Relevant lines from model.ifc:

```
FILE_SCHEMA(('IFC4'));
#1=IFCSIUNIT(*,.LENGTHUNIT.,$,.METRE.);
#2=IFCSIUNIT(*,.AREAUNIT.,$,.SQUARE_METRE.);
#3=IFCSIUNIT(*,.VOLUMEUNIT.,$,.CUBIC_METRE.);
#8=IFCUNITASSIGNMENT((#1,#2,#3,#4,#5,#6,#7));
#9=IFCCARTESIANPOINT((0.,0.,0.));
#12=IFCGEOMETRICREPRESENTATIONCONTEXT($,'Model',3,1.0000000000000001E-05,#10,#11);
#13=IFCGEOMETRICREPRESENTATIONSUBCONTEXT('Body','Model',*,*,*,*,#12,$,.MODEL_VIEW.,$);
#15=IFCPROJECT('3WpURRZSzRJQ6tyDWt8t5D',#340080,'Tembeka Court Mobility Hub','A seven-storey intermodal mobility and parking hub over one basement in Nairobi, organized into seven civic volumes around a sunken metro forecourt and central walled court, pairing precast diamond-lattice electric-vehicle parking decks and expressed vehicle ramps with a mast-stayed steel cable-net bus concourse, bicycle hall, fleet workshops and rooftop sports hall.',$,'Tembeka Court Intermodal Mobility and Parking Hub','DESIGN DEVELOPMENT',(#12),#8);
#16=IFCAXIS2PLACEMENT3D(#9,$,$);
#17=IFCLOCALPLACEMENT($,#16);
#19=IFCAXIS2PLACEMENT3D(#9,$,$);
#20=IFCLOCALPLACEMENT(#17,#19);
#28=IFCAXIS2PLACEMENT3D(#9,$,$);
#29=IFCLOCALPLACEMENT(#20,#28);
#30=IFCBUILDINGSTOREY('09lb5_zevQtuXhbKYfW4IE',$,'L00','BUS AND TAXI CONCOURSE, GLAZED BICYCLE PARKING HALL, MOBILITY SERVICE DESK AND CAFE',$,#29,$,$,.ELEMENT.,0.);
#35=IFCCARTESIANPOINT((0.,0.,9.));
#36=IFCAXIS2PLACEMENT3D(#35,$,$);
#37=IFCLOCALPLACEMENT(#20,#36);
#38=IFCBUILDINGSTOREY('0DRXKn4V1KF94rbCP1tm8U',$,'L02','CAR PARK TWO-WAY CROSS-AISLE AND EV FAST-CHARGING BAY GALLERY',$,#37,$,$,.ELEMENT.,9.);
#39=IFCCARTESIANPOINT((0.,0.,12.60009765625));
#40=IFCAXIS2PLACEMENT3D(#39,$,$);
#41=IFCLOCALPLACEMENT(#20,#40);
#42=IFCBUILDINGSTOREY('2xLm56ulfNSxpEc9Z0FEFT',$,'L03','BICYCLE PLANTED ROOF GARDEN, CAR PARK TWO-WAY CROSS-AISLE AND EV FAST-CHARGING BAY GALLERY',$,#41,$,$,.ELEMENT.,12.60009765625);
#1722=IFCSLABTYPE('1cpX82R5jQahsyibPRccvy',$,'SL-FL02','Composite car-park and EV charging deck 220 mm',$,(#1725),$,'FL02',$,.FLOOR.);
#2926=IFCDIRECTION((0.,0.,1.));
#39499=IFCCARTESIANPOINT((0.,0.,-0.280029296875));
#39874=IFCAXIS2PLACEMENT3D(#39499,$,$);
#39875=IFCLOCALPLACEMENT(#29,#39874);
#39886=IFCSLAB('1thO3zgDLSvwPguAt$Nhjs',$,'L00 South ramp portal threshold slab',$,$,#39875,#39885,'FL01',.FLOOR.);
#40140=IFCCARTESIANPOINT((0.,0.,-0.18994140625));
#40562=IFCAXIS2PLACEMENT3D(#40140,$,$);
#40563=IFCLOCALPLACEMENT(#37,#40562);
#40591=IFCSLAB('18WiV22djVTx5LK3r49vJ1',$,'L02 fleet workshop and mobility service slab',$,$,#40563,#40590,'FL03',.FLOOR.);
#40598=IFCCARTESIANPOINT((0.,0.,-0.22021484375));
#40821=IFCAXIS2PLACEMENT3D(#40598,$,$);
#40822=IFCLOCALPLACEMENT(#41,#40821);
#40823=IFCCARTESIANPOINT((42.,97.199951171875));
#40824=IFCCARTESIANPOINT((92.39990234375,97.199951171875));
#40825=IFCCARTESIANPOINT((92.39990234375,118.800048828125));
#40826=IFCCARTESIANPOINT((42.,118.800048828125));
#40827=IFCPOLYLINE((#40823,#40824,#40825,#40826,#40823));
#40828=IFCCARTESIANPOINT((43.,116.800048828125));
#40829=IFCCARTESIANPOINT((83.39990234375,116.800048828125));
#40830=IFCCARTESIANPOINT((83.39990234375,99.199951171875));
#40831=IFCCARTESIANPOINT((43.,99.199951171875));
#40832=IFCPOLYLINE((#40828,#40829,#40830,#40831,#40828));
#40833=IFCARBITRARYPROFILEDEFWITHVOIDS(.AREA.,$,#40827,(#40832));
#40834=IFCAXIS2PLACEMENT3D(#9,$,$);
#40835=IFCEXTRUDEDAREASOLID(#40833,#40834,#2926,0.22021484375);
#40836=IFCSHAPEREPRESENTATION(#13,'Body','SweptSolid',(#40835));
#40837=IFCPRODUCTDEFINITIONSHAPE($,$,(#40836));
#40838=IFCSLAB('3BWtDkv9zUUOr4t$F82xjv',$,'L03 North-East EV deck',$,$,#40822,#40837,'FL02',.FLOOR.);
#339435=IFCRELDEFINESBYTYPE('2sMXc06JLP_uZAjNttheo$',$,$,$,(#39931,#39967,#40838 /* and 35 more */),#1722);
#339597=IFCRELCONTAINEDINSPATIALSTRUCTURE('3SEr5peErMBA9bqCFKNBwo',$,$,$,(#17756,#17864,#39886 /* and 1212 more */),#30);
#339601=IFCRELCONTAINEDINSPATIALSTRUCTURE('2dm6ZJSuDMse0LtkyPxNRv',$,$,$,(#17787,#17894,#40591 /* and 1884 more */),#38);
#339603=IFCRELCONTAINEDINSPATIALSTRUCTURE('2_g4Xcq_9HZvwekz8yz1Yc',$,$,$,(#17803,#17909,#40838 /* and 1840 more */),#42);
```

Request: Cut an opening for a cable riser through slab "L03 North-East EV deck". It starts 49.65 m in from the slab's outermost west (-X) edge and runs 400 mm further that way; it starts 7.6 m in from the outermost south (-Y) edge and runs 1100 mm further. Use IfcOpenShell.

```python
import numpy as np
import ifcopenshell
import ifcopenshell.api.feature
import ifcopenshell.api.geometry
import ifcopenshell.api.root
import ifcopenshell.geom
import ifcopenshell.util.placement
import ifcopenshell.util.representation
import ifcopenshell.util.shape
import ifcopenshell.util.unit

model = ifcopenshell.open("model.ifc")
unit_scale = ifcopenshell.util.unit.calculate_unit_scale(model)
settings = ifcopenshell.geom.settings()


def volume(element):
    """Net volume in cubic metres, openings subtracted."""
    shape = ifcopenshell.geom.create_shape(settings, element)
    return ifcopenshell.util.shape.get_volume(shape.geometry)


slab = model.by_guid("3BWtDkv9zUUOr4t$F82xjv")
before = volume(slab)

# Extent in the slab's own axes, in metres. The edges named are its -X and -Y sides.
slab_shape = ifcopenshell.geom.create_shape(settings, slab)
vertices = ifcopenshell.util.shape.get_vertices(slab_shape.geometry)
x_min, y_min, bottom = vertices.min(axis=0)
top = vertices[:, 2].max()

opening = ifcopenshell.api.root.create_entity(model, ifc_class="IfcOpeningElement", name="Cable riser opening", predefined_type="OPENING")
context = ifcopenshell.util.representation.get_context(model, "Model", "Body", "MODEL_VIEW")
width, depth = 0.4, 1.1
outline = [(0.0, 0.0), (width, 0.0), (width, depth), (0.0, depth), (0.0, 0.0)]
# Overshoot both faces by 50 mm so the cut is clean.
shape = ifcopenshell.api.geometry.add_slab_representation(
    model, context=context, depth=top - bottom + 0.1, polyline=outline
)
ifcopenshell.api.geometry.assign_representation(model, product=opening, representation=shape)

matrix = ifcopenshell.util.placement.get_local_placement(slab.ObjectPlacement)
matrix[:, 3] = matrix @ np.append(np.array([x_min + 49.65, y_min + 7.6, bottom - 0.05]) / unit_scale, 1.0)
ifcopenshell.api.geometry.edit_object_placement(model, product=opening, matrix=matrix, is_si=False)
ifcopenshell.api.feature.add_feature(model, feature=opening, element=slab)

after = volume(slab)

print(f"slab volume {before:.3f} -> {after:.3f} m3")

model.write("model_updated.ifc")
```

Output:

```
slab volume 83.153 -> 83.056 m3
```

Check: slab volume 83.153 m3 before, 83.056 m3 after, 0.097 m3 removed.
